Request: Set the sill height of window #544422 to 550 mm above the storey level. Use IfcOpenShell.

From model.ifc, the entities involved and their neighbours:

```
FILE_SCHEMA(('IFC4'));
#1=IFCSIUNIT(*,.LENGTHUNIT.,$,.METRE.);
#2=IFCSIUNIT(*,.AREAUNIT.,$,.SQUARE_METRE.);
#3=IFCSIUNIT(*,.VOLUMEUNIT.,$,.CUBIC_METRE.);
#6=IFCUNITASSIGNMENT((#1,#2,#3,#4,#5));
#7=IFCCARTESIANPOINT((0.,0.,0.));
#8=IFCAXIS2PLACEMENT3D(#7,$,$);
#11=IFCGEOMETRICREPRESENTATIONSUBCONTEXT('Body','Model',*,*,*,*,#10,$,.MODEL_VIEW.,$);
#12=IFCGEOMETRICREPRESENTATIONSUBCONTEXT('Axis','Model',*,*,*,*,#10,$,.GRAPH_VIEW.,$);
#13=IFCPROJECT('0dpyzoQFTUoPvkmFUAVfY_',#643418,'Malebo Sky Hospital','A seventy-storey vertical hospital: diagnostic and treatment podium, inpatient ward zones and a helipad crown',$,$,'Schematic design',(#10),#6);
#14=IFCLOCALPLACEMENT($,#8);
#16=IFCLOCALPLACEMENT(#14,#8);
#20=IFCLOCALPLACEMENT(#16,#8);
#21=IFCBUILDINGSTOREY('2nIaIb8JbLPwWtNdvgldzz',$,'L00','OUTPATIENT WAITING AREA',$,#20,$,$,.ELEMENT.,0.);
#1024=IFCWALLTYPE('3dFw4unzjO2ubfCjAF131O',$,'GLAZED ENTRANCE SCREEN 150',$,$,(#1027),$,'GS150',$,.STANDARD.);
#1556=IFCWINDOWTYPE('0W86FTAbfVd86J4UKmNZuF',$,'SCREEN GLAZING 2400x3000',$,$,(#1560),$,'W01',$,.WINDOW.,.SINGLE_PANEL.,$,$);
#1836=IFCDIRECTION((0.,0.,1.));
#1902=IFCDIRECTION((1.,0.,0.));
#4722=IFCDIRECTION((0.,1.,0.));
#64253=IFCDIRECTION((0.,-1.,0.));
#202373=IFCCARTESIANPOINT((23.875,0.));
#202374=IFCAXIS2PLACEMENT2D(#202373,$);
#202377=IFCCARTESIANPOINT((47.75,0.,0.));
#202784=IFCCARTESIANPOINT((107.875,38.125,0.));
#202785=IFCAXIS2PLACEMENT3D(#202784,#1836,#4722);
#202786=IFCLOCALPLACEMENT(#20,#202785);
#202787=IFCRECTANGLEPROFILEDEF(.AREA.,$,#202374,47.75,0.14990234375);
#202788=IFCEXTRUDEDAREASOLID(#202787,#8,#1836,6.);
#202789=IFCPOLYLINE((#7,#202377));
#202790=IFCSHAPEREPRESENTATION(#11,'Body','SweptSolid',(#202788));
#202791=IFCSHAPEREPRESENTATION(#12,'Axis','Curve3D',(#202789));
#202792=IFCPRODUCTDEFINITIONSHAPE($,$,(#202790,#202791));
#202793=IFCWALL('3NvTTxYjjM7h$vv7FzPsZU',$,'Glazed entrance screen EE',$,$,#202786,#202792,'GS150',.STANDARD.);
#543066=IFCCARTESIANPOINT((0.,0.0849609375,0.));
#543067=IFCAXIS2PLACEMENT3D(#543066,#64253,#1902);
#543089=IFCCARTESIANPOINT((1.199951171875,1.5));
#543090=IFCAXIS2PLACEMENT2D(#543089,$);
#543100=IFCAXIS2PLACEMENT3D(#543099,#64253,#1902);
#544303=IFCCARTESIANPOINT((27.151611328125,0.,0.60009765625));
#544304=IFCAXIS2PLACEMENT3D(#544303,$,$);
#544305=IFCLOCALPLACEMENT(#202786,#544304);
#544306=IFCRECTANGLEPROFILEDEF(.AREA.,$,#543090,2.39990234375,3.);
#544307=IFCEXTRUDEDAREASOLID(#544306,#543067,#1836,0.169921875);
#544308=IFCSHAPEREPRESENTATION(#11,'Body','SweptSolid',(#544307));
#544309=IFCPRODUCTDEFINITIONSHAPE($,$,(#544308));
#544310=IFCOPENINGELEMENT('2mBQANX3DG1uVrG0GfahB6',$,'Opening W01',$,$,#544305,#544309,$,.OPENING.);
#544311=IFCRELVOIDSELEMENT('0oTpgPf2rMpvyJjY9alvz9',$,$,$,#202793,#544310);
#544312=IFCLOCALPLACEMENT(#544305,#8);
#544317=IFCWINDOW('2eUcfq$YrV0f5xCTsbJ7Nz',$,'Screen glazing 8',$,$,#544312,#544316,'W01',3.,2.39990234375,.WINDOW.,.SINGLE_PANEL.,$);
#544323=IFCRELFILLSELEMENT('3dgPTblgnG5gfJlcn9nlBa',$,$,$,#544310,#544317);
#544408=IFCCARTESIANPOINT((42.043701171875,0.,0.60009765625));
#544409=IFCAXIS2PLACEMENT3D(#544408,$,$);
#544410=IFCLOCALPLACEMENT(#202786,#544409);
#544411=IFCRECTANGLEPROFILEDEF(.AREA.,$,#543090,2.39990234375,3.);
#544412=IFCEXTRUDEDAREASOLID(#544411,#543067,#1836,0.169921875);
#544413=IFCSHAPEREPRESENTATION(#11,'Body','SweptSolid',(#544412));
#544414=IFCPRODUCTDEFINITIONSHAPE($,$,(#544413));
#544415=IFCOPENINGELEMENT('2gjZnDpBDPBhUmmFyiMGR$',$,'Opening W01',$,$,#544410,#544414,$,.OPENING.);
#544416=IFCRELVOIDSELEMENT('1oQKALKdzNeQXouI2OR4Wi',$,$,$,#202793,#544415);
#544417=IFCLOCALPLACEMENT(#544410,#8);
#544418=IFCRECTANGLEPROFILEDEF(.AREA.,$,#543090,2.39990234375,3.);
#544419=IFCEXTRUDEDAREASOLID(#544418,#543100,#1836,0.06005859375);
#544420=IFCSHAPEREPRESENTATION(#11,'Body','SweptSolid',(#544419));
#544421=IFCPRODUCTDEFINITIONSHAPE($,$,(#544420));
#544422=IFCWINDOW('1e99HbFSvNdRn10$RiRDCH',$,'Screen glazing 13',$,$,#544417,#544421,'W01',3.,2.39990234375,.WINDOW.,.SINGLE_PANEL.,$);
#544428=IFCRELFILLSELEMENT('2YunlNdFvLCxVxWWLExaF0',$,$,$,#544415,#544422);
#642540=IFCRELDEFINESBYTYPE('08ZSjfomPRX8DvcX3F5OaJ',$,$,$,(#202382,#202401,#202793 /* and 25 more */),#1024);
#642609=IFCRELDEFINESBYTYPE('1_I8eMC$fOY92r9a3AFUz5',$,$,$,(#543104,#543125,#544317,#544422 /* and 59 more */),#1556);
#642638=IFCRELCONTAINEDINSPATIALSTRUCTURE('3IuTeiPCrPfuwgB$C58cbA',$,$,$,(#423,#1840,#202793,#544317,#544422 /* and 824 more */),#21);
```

```python
import numpy as np
import ifcopenshell
import ifcopenshell.api.geometry
import ifcopenshell.geom
import ifcopenshell.util.element
import ifcopenshell.util.placement
import ifcopenshell.util.shape
import ifcopenshell.util.unit

model = ifcopenshell.open("model.ifc")
unit_scale = ifcopenshell.util.unit.calculate_unit_scale(model)

window = model.by_id(544422)
opening = window.FillsVoids[0].RelatingOpeningElement
storey = ifcopenshell.util.element.get_container(window, ifc_class="IfcBuildingStorey")
level = ifcopenshell.util.placement.get_local_placement(storey.ObjectPlacement)[2, 3]

# The opening's origin need not be at the sill, so measure its lowest point.
shape = ifcopenshell.geom.create_shape(ifcopenshell.geom.settings(), opening)
bottom = ifcopenshell.util.shape.get_shape_bottom_elevation(shape, shape.geometry) / unit_scale
dz = level + 0.55 / unit_scale - bottom

shift = np.array([0.0, 0.0, dz])
# The window is placed relative to its opening, so it follows when the opening moves.
matrix = ifcopenshell.util.placement.get_local_placement(opening.ObjectPlacement)
matrix[:3, 3] += shift
ifcopenshell.api.geometry.edit_object_placement(
    model, product=opening, matrix=matrix, is_si=False, should_transform_children=True
)

print(f"moved by {dz * unit_scale:+.3f} m")

model.write("model_updated.ifc")
```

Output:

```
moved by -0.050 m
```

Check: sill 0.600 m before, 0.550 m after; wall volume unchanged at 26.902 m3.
